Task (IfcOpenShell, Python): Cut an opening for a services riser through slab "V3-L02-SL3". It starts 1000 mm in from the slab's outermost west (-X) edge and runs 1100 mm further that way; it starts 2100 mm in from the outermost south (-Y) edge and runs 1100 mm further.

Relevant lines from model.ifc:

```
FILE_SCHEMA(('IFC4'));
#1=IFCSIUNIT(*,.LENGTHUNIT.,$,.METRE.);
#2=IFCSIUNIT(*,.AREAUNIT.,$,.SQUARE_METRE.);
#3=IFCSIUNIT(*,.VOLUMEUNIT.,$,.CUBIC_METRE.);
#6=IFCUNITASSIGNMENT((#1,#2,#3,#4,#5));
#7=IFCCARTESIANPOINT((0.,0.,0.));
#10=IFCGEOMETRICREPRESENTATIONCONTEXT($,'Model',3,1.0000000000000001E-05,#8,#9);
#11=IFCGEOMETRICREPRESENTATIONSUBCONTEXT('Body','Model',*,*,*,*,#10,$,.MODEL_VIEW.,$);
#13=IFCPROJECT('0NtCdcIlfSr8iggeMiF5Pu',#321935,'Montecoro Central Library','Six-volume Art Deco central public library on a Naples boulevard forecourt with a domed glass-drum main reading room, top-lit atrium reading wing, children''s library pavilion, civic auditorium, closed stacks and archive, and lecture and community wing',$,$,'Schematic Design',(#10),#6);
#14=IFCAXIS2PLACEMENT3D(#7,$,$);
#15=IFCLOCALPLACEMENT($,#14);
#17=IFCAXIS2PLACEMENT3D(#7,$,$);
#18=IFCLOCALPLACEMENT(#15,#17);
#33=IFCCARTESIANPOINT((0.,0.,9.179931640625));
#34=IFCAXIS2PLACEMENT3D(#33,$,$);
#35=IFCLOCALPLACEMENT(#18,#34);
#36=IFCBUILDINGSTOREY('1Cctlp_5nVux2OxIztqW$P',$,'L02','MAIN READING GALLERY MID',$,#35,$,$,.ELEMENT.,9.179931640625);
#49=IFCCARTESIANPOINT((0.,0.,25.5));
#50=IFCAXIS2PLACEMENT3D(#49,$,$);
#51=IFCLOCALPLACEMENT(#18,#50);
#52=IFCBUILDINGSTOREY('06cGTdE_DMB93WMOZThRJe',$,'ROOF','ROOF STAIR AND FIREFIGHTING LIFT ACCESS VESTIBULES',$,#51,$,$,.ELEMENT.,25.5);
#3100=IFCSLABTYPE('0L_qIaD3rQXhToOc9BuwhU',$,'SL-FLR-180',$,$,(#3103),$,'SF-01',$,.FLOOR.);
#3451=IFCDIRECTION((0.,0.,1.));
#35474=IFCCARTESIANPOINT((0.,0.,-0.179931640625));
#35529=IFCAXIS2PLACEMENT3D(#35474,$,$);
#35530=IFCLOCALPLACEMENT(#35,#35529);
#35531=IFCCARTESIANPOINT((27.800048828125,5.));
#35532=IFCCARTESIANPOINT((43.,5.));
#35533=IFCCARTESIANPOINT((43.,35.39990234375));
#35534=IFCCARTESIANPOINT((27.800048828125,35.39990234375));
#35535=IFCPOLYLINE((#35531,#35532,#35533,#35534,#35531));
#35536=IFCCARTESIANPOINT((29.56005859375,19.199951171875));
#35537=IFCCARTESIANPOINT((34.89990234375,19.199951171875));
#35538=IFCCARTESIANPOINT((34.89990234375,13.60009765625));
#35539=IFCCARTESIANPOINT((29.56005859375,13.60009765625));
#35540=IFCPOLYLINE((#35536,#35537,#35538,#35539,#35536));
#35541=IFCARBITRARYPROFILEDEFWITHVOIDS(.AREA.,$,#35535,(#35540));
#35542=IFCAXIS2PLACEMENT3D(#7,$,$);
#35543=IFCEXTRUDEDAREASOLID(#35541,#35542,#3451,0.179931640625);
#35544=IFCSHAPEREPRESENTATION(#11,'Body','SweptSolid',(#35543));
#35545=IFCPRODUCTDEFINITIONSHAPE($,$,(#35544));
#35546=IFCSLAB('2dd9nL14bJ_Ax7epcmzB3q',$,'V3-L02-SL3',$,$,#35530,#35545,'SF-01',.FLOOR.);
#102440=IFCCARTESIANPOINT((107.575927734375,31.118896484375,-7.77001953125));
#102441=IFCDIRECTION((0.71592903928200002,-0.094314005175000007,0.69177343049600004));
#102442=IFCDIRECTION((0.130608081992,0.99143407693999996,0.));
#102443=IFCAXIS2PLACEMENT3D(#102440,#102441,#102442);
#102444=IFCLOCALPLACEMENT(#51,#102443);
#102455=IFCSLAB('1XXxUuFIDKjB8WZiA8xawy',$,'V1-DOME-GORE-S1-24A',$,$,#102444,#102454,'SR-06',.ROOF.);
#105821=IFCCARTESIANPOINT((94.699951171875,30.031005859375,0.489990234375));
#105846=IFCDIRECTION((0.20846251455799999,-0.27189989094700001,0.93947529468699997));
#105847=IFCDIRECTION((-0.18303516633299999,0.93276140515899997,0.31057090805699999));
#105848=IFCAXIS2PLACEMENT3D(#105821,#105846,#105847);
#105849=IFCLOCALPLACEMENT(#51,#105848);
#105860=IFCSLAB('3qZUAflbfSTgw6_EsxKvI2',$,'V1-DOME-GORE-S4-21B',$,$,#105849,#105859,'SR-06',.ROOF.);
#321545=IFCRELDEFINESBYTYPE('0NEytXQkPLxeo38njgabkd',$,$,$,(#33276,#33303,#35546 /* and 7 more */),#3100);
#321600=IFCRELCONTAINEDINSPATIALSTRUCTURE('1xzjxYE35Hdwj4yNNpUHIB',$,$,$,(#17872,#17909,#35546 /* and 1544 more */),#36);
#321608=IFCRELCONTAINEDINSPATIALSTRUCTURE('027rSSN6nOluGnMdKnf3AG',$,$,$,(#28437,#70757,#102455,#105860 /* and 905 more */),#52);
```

```python
import numpy as np
import ifcopenshell
import ifcopenshell.api.feature
import ifcopenshell.api.geometry
import ifcopenshell.api.root
import ifcopenshell.geom
import ifcopenshell.util.placement
import ifcopenshell.util.representation
import ifcopenshell.util.shape
import ifcopenshell.util.unit

model = ifcopenshell.open("model.ifc")
unit_scale = ifcopenshell.util.unit.calculate_unit_scale(model)
settings = ifcopenshell.geom.settings()


def volume(element):
    """Net volume in cubic metres, openings subtracted."""
    shape = ifcopenshell.geom.create_shape(settings, element)
    return ifcopenshell.util.shape.get_volume(shape.geometry)


slab = model.by_guid("2dd9nL14bJ_Ax7epcmzB3q")
before = volume(slab)

# Extent in the slab's own axes, in metres. The edges named are its -X and -Y sides.
slab_shape = ifcopenshell.geom.create_shape(settings, slab)
vertices = ifcopenshell.util.shape.get_vertices(slab_shape.geometry)
x_min, y_min, bottom = vertices.min(axis=0)
top = vertices[:, 2].max()

opening = ifcopenshell.api.root.create_entity(model, ifc_class="IfcOpeningElement", name="Services riser opening", predefined_type="OPENING")
context = ifcopenshell.util.representation.get_context(model, "Model", "Body", "MODEL_VIEW")
width, depth = 1.1, 1.1
outline = [(0.0, 0.0), (width, 0.0), (width, depth), (0.0, depth), (0.0, 0.0)]
# Overshoot both faces by 50 mm so the cut is clean.
shape = ifcopenshell.api.geometry.add_slab_representation(
    model, context=context, depth=top - bottom + 0.1, polyline=outline
)
ifcopenshell.api.geometry.assign_representation(model, product=opening, representation=shape)

matrix = ifcopenshell.util.placement.get_local_placement(slab.ObjectPlacement)
matrix[:, 3] = matrix @ np.append(np.array([x_min + 1, y_min + 2.1, bottom - 0.05]) / unit_scale, 1.0)
ifcopenshell.api.geometry.edit_object_placement(model, product=opening, matrix=matrix, is_si=False)
ifcopenshell.api.feature.add_feature(model, feature=opening, element=slab)

after = volume(slab)

print(f"slab volume {before:.3f} -> {after:.3f} m3")

model.write("model_updated.ifc")
```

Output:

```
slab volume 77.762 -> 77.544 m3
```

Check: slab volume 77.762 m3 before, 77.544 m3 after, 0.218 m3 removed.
